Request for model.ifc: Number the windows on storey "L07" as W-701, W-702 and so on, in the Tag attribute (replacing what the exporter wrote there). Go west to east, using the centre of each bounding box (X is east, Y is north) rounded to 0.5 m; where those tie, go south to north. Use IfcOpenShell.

First a look at what the model holds.

```python
import ifcopenshell
import ifcopenshell.util.element
import ifcopenshell.util.placement

model = ifcopenshell.open("model.ifc")
print(model.schema)
storey = next(s for s in model.by_type("IfcBuildingStorey") if s.Name == "L07")
windows = [e for e in ifcopenshell.util.element.get_decomposition(storey) if e.is_a("IfcWindow")]
for e in sorted(windows, key=lambda e: e.id()):
    origin = ifcopenshell.util.placement.get_local_placement(e.ObjectPlacement)[:3, 3]
    print(e.id(), e.Tag, e.Name, origin.round(2) + 0.0, sep=" | ")
```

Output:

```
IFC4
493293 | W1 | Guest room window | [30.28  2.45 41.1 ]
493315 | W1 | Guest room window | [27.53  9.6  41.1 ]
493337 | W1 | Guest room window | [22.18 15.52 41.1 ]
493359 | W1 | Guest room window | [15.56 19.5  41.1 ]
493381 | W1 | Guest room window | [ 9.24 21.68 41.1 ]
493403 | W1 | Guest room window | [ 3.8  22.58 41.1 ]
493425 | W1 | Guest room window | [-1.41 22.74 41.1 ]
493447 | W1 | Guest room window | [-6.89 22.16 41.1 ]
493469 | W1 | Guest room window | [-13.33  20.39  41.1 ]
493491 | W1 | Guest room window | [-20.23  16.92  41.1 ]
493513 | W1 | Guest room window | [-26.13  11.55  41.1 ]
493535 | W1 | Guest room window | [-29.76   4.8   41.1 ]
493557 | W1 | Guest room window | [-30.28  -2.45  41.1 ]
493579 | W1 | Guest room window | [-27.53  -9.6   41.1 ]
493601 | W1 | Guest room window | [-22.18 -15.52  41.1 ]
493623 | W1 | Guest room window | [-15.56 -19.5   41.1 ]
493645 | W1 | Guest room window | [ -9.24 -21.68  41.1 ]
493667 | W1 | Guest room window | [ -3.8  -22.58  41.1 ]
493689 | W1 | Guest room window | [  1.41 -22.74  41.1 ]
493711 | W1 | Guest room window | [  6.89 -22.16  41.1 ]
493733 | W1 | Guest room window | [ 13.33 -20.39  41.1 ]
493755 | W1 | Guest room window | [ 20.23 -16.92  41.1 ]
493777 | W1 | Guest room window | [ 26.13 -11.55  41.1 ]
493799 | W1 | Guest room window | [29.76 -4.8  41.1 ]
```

```python
import ifcopenshell
import ifcopenshell.geom
import ifcopenshell.util.element
import ifcopenshell.util.shape

model = ifcopenshell.open("model.ifc")
settings = ifcopenshell.geom.settings()
settings.set("use-world-coords", True)


def centre(element):
    shape = ifcopenshell.geom.create_shape(settings, element)
    return ifcopenshell.util.shape.get_bbox_centroid(shape.geometry)


storey = next(s for s in model.by_type("IfcBuildingStorey") if s.Name == "L07")
windows = [e for e in ifcopenshell.util.element.get_decomposition(storey) if e.is_a("IfcWindow")]

# Insertion points can sit at a corner or the storey origin, so sort by the geometry (in metres).
centres = {e: centre(e) for e in windows}
windows.sort(key=lambda e: (round(centres[e][0] / 0.5), centres[e][1]))

for i, e in enumerate(windows, start=1):
    number = f"W-7{i:02d}"
    e.Tag = number
    print(e.id(), number)

model.write("model_rev.ifc")
```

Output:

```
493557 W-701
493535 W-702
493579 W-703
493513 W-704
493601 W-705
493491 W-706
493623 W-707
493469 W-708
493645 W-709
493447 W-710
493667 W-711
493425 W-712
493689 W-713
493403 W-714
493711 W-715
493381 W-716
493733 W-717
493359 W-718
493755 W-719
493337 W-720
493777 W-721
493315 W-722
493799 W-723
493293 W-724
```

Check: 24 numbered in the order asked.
